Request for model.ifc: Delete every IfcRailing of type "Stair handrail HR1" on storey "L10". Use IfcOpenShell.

First a look at what the model holds.

```python
import ifcopenshell
import ifcopenshell.util.element

model = ifcopenshell.open("model.ifc")
print(model.schema)
storey = next(s for s in model.by_type("IfcBuildingStorey") if s.Name == "L10")
railings = [e for e in ifcopenshell.util.element.get_decomposition(storey) if e.is_a("IfcRailing")]
seen = {}
for e in railings:
    element_type = ifcopenshell.util.element.get_type(e)
    name = element_type.Name if element_type not in (None, e) else None
    seen[name] = seen.get(name, 0) + 1
for name, count in sorted(seen.items(), key=str):
    print(count, "x", name)
```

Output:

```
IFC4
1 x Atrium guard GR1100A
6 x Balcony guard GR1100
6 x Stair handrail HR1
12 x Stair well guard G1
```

```python
import ifcopenshell
import ifcopenshell.api.root
import ifcopenshell.util.element

model = ifcopenshell.open("model.ifc")

storey = next(s for s in model.by_type("IfcBuildingStorey") if s.Name == "L10")
railings = [e for e in ifcopenshell.util.element.get_decomposition(storey) if e.is_a("IfcRailing")]
targets = [e for e in railings if (t := ifcopenshell.util.element.get_type(e)) not in (None, e) and t.Name == "Stair handrail HR1"]

for e in targets:
    ifcopenshell.api.root.remove_product(model, product=e)
print(len(targets), "removed")

model.write("model_updated.ifc")
```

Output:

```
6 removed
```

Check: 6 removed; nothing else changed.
